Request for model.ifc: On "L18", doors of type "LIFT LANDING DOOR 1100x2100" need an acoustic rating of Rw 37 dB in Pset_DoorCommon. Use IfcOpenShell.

First a look at what the model holds.

```python
import ifcopenshell
import ifcopenshell.util.element

model = ifcopenshell.open("model.ifc")
print(model.schema)
storey = next(s for s in model.by_type("IfcBuildingStorey") if s.Name == "L18")
doors = [e for e in ifcopenshell.util.element.get_decomposition(storey) if e.is_a("IfcDoor")]
seen = {}
for e in doors:
    element_type = ifcopenshell.util.element.get_type(e)
    key = (element_type.Name if element_type != e and element_type else None, ifcopenshell.util.element.get_pset(e, "Pset_DoorCommon", "AcousticRating"))
    seen[key] = seen.get(key, 0) + 1
for (name, value), count in sorted(seen.items(), key=str):
    print(count, "x", name, "|", value)
```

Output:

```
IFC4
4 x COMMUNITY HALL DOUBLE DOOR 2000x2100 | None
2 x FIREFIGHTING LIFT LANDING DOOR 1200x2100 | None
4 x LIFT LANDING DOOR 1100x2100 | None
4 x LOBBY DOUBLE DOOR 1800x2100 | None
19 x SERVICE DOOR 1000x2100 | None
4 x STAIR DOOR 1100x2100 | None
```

```python
import ifcopenshell
import ifcopenshell.api.pset
import ifcopenshell.util.element

model = ifcopenshell.open("model.ifc")

storey = next(s for s in model.by_type("IfcBuildingStorey") if s.Name == "L18")
doors = [e for e in ifcopenshell.util.element.get_decomposition(storey) if e.is_a("IfcDoor")]

count = 0
for e in doors:
    element_type = ifcopenshell.util.element.get_type(e)
    if element_type in (None, e) or element_type.Name != "LIFT LANDING DOOR 1100x2100":
        continue
    found = ifcopenshell.util.element.get_pset(e, "Pset_DoorCommon", should_inherit=False)
    if found:
        pset = model.by_id(found["id"])
        if len(ifcopenshell.util.element.get_elements_by_pset(pset)) > 1:
            pset = ifcopenshell.api.pset.unshare_pset(model, products=[e], pset=pset)[0]
    else:
        pset = ifcopenshell.api.pset.add_pset(model, product=e, name="Pset_DoorCommon")
    ifcopenshell.api.pset.edit_pset(model, pset=pset, properties={"AcousticRating": "Rw 37 dB"})
    count += 1

print(count, "doors updated")

model.write("model_rev.ifc")
```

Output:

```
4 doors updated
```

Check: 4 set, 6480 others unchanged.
